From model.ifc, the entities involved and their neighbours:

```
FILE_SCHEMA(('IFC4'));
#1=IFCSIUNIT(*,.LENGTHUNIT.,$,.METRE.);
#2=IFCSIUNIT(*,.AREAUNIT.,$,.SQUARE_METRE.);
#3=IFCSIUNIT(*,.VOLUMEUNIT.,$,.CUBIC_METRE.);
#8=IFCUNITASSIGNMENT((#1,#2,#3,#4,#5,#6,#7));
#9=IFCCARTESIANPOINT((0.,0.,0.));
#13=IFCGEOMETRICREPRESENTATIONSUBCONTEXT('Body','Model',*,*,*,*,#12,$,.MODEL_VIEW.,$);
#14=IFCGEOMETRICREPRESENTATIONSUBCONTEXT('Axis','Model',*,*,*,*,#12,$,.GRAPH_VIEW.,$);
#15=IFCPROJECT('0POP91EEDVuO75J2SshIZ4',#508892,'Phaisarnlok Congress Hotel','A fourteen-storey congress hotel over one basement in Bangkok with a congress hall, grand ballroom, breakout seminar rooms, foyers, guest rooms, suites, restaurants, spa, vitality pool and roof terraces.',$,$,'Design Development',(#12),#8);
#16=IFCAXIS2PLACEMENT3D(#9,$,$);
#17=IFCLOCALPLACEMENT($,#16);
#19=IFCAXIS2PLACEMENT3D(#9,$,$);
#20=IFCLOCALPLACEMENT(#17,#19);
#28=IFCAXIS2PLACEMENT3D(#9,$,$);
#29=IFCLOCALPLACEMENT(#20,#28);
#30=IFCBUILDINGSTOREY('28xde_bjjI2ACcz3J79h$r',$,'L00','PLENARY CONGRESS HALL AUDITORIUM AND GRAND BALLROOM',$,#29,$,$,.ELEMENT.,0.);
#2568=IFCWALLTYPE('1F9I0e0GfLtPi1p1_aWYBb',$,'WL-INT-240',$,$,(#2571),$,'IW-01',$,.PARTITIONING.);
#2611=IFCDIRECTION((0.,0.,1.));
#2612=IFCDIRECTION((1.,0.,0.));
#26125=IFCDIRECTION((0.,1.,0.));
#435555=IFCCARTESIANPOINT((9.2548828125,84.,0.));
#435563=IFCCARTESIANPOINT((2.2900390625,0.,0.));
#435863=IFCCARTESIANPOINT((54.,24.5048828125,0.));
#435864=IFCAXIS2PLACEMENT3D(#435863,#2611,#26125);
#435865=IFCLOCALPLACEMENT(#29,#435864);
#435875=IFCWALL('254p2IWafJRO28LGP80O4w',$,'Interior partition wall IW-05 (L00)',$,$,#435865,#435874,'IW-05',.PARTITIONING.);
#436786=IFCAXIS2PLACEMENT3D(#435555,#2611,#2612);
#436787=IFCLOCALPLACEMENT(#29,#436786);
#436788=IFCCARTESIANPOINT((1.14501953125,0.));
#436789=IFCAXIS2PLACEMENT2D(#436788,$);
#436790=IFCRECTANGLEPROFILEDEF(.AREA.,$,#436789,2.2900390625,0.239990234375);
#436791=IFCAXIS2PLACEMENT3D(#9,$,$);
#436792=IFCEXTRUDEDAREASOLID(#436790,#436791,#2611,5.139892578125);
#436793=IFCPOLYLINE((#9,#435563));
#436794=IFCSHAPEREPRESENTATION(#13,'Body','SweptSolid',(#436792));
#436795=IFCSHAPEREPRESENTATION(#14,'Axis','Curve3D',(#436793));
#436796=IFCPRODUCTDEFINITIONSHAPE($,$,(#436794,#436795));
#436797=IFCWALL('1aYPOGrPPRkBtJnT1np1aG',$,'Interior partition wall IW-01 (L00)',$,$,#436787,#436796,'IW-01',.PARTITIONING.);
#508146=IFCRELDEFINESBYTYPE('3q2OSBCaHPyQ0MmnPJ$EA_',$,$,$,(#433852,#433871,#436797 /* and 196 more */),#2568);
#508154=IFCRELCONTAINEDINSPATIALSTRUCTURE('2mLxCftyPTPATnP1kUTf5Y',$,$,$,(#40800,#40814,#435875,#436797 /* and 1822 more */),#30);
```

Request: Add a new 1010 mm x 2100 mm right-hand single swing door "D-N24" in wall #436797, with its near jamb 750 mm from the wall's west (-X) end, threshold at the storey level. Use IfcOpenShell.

```python
import numpy as np
import ifcopenshell
import ifcopenshell.api.feature
import ifcopenshell.api.geometry
import ifcopenshell.api.root
import ifcopenshell.api.spatial
import ifcopenshell.geom
import ifcopenshell.util.element
import ifcopenshell.util.placement
import ifcopenshell.util.representation
import ifcopenshell.util.shape
import ifcopenshell.util.unit

model = ifcopenshell.open("model.ifc")
unit_scale = ifcopenshell.util.unit.calculate_unit_scale(model)
settings = ifcopenshell.geom.settings()


def volume(element):
    """Net volume in cubic metres, openings subtracted."""
    shape = ifcopenshell.geom.create_shape(settings, element)
    return ifcopenshell.util.shape.get_volume(shape.geometry)


wall = model.by_guid("1aYPOGrPPRkBtJnT1np1aG")
storey = ifcopenshell.util.element.get_container(wall, ifc_class="IfcBuildingStorey")
context = ifcopenshell.util.representation.get_context(model, "Model", "Body", "MODEL_VIEW")
before = volume(wall)

width, height, from_end, sill = 1.01, 2.1, 0.75, 0.0  # metres

# The wall runs along its own X axis, and the end named is its -X end.
wall_shape = ifcopenshell.geom.create_shape(settings, wall)
x, y, z = ifcopenshell.util.shape.get_vertices(wall_shape.geometry).T
start = x.min() + from_end
face, thickness = float(y.min()), float(y.max() - y.min())
wall_matrix = ifcopenshell.util.placement.get_local_placement(wall.ObjectPlacement)
level = ifcopenshell.util.placement.get_local_placement(storey.ObjectPlacement)[2, 3]


def in_wall(x, y):
    """Placement at x, y metres in the wall's axes, at sill height."""
    matrix = wall_matrix.copy()
    matrix[:, 3] = wall_matrix @ np.array([x / unit_scale, y / unit_scale, 0.0, 1.0])
    matrix[2, 3] = level + sill / unit_scale
    return matrix


# Opening: a box that overshoots both wall faces by 50 mm.
opening = ifcopenshell.api.root.create_entity(model, ifc_class="IfcOpeningElement", predefined_type="OPENING")
box = ifcopenshell.api.geometry.add_wall_representation(
    model, context=context, length=width, height=height, thickness=thickness + 0.1
)
ifcopenshell.api.geometry.assign_representation(model, product=opening, representation=box)
ifcopenshell.api.geometry.edit_object_placement(model, product=opening, matrix=in_wall(start, face - 0.05), is_si=False)
ifcopenshell.api.feature.add_feature(model, feature=opening, element=wall)

door = ifcopenshell.api.root.create_entity(model, ifc_class="IfcDoor", name="D-N24", predefined_type="DOOR")
door.OverallWidth, door.OverallHeight = width / unit_scale, height / unit_scale
door.OperationType = "SINGLE_SWING_RIGHT"
body = ifcopenshell.api.geometry.add_door_representation(
    model,
    context=context,
    overall_width=door.OverallWidth,
    overall_height=door.OverallHeight,
    operation_type="SINGLE_SWING_RIGHT",
    lining_properties={"LiningDepth": thickness / unit_scale, "ThresholdDepth": thickness / unit_scale},
)
ifcopenshell.api.geometry.assign_representation(model, product=door, representation=body)
ifcopenshell.api.spatial.assign_container(model, products=[door], relating_structure=storey)
ifcopenshell.api.feature.add_filling(model, opening=opening, element=door)

# The lining spans the wall, so the door starts at the wall face.
ifcopenshell.api.geometry.edit_object_placement(model, product=door, matrix=in_wall(start, face), is_si=False)

after = volume(wall)

print(f"wall volume {before:.3f} -> {after:.3f} m3")

model.write("model-out.ifc")
```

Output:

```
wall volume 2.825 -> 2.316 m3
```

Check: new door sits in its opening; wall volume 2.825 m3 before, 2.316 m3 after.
